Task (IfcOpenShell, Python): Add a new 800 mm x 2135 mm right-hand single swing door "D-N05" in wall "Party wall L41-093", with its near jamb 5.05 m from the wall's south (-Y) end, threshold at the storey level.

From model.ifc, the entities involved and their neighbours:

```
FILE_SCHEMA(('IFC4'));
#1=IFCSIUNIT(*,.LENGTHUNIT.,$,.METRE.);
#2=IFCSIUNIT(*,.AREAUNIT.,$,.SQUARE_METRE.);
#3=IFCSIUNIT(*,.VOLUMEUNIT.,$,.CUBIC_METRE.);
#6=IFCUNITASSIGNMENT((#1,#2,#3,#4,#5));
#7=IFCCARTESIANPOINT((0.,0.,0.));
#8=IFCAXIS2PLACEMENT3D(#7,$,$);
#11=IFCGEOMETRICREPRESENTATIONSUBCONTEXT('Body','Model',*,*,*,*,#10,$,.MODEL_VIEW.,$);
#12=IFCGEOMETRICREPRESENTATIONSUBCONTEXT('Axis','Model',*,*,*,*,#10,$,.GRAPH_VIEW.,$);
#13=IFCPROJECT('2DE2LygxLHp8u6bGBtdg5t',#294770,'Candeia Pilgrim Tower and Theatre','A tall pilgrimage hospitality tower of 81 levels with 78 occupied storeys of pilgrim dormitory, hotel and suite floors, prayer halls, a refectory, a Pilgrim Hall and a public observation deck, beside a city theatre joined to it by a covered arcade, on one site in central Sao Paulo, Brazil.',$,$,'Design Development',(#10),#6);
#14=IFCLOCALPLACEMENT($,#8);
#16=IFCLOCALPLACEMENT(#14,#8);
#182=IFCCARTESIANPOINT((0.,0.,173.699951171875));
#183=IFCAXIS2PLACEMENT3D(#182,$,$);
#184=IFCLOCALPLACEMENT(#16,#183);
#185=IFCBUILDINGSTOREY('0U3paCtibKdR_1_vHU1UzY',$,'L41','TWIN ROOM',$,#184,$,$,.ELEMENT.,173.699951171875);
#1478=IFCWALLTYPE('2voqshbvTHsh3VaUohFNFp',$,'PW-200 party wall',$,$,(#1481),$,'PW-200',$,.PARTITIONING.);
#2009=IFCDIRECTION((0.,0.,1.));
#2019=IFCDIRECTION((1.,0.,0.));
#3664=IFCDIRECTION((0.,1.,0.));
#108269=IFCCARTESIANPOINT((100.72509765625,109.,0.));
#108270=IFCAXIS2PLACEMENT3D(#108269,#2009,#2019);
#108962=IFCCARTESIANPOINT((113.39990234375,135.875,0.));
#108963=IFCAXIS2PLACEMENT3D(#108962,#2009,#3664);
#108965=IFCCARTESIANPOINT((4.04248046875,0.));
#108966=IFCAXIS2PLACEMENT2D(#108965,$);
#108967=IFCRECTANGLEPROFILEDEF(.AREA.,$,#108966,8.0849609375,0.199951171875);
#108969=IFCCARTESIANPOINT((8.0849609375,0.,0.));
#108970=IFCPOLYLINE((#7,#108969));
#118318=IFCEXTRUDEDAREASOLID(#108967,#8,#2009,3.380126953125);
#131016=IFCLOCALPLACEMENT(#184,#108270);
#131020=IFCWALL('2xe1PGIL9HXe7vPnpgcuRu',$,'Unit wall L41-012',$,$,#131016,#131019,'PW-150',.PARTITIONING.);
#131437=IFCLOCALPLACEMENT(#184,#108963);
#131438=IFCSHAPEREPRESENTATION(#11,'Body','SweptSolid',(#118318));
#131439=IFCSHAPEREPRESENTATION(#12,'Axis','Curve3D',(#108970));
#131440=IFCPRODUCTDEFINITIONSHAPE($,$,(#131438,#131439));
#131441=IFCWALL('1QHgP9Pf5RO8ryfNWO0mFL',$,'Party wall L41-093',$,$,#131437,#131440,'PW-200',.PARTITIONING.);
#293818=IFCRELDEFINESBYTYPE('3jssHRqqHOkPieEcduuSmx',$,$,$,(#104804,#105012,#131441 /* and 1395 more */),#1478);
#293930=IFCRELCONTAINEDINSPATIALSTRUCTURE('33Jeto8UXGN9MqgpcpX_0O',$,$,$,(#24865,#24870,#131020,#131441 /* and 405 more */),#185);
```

```python
import numpy as np
import ifcopenshell
import ifcopenshell.api.feature
import ifcopenshell.api.geometry
import ifcopenshell.api.root
import ifcopenshell.api.spatial
import ifcopenshell.geom
import ifcopenshell.util.element
import ifcopenshell.util.placement
import ifcopenshell.util.representation
import ifcopenshell.util.shape
import ifcopenshell.util.unit

model = ifcopenshell.open("model.ifc")
unit_scale = ifcopenshell.util.unit.calculate_unit_scale(model)
settings = ifcopenshell.geom.settings()


def volume(element):
    """Net volume in cubic metres, openings subtracted."""
    shape = ifcopenshell.geom.create_shape(settings, element)
    return ifcopenshell.util.shape.get_volume(shape.geometry)


wall = model.by_id(131441)
storey = ifcopenshell.util.element.get_container(wall, ifc_class="IfcBuildingStorey")
context = ifcopenshell.util.representation.get_context(model, "Model", "Body", "MODEL_VIEW")
before = volume(wall)

width, height, from_end, sill = 0.8, 2.135, 5.05, 0.0  # metres

# The wall runs along its own X axis, and the end named is its -X end.
wall_shape = ifcopenshell.geom.create_shape(settings, wall)
x, y, z = ifcopenshell.util.shape.get_vertices(wall_shape.geometry).T
start = x.min() + from_end
face, thickness = float(y.min()), float(y.max() - y.min())
wall_matrix = ifcopenshell.util.placement.get_local_placement(wall.ObjectPlacement)
level = ifcopenshell.util.placement.get_local_placement(storey.ObjectPlacement)[2, 3]


def in_wall(x, y):
    """Placement at x, y metres in the wall's axes, at sill height."""
    matrix = wall_matrix.copy()
    matrix[:, 3] = wall_matrix @ np.array([x / unit_scale, y / unit_scale, 0.0, 1.0])
    matrix[2, 3] = level + sill / unit_scale
    return matrix


# Opening: a box that overshoots both wall faces by 50 mm.
opening = ifcopenshell.api.root.create_entity(model, ifc_class="IfcOpeningElement", predefined_type="OPENING")
box = ifcopenshell.api.geometry.add_wall_representation(
    model, context=context, length=width, height=height, thickness=thickness + 0.1
)
ifcopenshell.api.geometry.assign_representation(model, product=opening, representation=box)
ifcopenshell.api.geometry.edit_object_placement(model, product=opening, matrix=in_wall(start, face - 0.05), is_si=False)
ifcopenshell.api.feature.add_feature(model, feature=opening, element=wall)

door = ifcopenshell.api.root.create_entity(model, ifc_class="IfcDoor", name="D-N05", predefined_type="DOOR")
door.OverallWidth, door.OverallHeight = width / unit_scale, height / unit_scale
door.OperationType = "SINGLE_SWING_RIGHT"
body = ifcopenshell.api.geometry.add_door_representation(
    model,
    context=context,
    overall_width=door.OverallWidth,
    overall_height=door.OverallHeight,
    operation_type="SINGLE_SWING_RIGHT",
    lining_properties={"LiningDepth": thickness / unit_scale, "ThresholdDepth": thickness / unit_scale},
)
ifcopenshell.api.geometry.assign_representation(model, product=door, representation=body)
ifcopenshell.api.spatial.assign_container(model, products=[door], relating_structure=storey)
ifcopenshell.api.feature.add_filling(model, opening=opening, element=door)

# The lining spans the wall, so the door starts at the wall face.
ifcopenshell.api.geometry.edit_object_placement(model, product=door, matrix=in_wall(start, face), is_si=False)

after = volume(wall)

print(f"wall volume {before:.3f} -> {after:.3f} m3")

model.write("model-out.ifc")
```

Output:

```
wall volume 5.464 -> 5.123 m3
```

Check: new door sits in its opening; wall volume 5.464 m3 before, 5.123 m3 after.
